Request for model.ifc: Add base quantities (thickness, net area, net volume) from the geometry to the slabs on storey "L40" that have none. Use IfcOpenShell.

First a look at what the model holds.

```python
import ifcopenshell
import ifcopenshell.util.element
import ifcopenshell.util.unit

model = ifcopenshell.open("model.ifc")
print(model.schema)
for unit_type in ("LENGTHUNIT", "AREAUNIT", "VOLUMEUNIT"):
    print(unit_type, ifcopenshell.util.unit.calculate_unit_scale(model, unit_type))
storey = next(s for s in model.by_type("IfcBuildingStorey") if s.Name == "L40")
slabs = [e for e in ifcopenshell.util.element.get_decomposition(storey) if e.is_a("IfcSlab")]
for e in sorted(slabs, key=lambda e: e.id()):
    print(e.id(), e.is_a(), e.Name, list(ifcopenshell.util.element.get_psets(e, qtos_only=True)), sep=" | ")
```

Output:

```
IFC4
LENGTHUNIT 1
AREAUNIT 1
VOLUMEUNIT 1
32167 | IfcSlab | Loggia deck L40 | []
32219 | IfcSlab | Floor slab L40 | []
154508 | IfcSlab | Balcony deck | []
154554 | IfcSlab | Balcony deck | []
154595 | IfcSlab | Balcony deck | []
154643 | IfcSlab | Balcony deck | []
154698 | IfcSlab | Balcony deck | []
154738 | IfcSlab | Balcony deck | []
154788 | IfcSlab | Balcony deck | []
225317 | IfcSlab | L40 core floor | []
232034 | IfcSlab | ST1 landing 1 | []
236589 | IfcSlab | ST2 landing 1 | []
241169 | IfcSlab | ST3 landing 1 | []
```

```python
import ifcopenshell
import ifcopenshell.api.pset
import ifcopenshell.geom
import ifcopenshell.util.element
import ifcopenshell.util.shape
import ifcopenshell.util.unit

model = ifcopenshell.open("model.ifc")
unit_scale = ifcopenshell.util.unit.calculate_unit_scale(model)
area_scale = ifcopenshell.util.unit.calculate_unit_scale(model, "AREAUNIT")
volume_scale = ifcopenshell.util.unit.calculate_unit_scale(model, "VOLUMEUNIT")
settings = ifcopenshell.geom.settings()

storey = next(s for s in model.by_type("IfcBuildingStorey") if s.Name == "L40")
slabs = [e for e in ifcopenshell.util.element.get_decomposition(storey) if e.is_a("IfcSlab")]

for e in sorted(slabs, key=lambda e: e.id()):
    if ifcopenshell.util.element.get_psets(e, qtos_only=True, should_inherit=False):
        continue
    # Geometry comes back in metres, in the element's own axes.
    shape = ifcopenshell.geom.create_shape(settings, e)
    values = {
        "Width": ifcopenshell.util.shape.get_z(shape.geometry) / unit_scale,
        "NetArea": ifcopenshell.util.shape.get_footprint_area(shape.geometry) / area_scale,
        "NetVolume": ifcopenshell.util.shape.get_volume(shape.geometry) / volume_scale,
    }
    qto = ifcopenshell.api.pset.add_qto(model, product=e, name="Qto_SlabBaseQuantities")
    ifcopenshell.api.pset.edit_qto(model, qto=qto, properties=values)
    print(e.id(), {k: round(v, 3) for k, v in values.items()})

model.write("model_edited.ifc")
```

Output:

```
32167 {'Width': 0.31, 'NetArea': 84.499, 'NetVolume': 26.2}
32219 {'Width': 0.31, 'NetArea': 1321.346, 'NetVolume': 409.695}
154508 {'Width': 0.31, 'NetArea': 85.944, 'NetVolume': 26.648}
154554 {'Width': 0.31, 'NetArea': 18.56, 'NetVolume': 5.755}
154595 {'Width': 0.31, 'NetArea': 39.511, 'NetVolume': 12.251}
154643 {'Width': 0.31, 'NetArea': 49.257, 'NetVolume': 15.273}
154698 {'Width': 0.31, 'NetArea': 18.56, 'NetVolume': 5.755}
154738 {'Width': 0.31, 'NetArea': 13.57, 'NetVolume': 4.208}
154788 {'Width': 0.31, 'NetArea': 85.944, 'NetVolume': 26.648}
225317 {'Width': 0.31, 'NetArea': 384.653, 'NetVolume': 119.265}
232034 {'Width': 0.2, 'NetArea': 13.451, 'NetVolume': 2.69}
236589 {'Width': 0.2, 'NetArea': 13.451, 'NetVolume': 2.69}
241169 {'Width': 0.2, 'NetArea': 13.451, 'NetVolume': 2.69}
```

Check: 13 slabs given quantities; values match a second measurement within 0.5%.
